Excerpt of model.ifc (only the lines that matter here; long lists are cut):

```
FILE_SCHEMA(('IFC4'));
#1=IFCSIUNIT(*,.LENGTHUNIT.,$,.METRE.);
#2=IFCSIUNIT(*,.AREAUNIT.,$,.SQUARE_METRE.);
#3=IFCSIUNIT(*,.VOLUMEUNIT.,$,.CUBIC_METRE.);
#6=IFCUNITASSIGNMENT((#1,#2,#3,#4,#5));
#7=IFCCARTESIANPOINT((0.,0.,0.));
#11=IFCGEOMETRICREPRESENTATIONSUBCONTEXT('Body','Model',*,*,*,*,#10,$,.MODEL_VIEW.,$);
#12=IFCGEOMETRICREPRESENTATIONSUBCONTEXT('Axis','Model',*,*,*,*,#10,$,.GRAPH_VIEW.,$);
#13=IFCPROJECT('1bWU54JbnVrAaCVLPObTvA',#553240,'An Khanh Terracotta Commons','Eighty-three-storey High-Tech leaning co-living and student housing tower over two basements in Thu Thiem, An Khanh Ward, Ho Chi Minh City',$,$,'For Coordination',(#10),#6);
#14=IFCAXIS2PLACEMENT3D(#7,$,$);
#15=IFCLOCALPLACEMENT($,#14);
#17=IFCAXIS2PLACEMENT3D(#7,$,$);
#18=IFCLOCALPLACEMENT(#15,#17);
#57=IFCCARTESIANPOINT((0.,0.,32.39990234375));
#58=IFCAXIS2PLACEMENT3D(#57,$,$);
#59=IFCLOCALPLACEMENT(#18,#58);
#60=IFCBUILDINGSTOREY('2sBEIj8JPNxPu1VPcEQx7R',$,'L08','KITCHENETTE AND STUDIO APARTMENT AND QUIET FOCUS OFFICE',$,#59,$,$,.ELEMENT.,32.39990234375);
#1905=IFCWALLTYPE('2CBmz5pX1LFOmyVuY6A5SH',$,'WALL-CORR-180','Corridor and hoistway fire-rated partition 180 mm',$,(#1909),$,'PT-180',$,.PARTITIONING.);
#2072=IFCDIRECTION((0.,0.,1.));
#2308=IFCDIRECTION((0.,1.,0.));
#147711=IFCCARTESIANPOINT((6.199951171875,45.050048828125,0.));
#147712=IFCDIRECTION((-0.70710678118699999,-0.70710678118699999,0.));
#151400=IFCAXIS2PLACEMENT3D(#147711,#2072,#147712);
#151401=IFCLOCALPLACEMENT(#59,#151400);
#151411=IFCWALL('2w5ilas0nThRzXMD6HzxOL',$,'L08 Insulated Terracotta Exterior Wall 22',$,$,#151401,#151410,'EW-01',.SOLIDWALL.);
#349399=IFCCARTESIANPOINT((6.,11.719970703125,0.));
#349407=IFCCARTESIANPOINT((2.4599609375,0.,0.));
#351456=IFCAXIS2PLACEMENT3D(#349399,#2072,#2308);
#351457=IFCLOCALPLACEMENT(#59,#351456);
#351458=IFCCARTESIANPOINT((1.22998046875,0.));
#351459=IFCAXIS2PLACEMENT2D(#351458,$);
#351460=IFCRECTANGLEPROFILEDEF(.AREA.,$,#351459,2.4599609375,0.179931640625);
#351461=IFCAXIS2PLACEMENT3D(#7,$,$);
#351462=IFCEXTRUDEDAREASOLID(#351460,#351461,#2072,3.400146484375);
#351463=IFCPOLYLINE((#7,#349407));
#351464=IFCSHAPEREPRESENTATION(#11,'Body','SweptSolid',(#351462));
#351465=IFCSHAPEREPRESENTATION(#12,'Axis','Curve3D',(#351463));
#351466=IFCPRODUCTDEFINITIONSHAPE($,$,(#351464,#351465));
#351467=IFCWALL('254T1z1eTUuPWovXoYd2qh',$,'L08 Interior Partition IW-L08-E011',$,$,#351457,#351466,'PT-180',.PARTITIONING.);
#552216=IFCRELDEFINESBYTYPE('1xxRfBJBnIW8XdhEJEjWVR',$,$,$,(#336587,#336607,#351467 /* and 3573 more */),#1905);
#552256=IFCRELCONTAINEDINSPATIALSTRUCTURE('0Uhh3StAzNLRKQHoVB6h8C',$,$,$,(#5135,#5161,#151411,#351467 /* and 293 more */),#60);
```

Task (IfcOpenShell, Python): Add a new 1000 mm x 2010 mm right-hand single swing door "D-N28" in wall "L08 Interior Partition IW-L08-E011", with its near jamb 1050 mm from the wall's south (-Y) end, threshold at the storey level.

```python
import numpy as np
import ifcopenshell
import ifcopenshell.api.feature
import ifcopenshell.api.geometry
import ifcopenshell.api.root
import ifcopenshell.api.spatial
import ifcopenshell.geom
import ifcopenshell.util.element
import ifcopenshell.util.placement
import ifcopenshell.util.representation
import ifcopenshell.util.shape
import ifcopenshell.util.unit

model = ifcopenshell.open("model.ifc")
unit_scale = ifcopenshell.util.unit.calculate_unit_scale(model)
settings = ifcopenshell.geom.settings()


def volume(element):
    """Net volume in cubic metres, openings subtracted."""
    shape = ifcopenshell.geom.create_shape(settings, element)
    return ifcopenshell.util.shape.get_volume(shape.geometry)


wall = model.by_guid("254T1z1eTUuPWovXoYd2qh")
storey = ifcopenshell.util.element.get_container(wall, ifc_class="IfcBuildingStorey")
context = ifcopenshell.util.representation.get_context(model, "Model", "Body", "MODEL_VIEW")
before = volume(wall)

width, height, from_end, sill = 1, 2.01, 1.05, 0.0  # metres

# The wall runs along its own X axis, and the end named is its -X end.
wall_shape = ifcopenshell.geom.create_shape(settings, wall)
x, y, z = ifcopenshell.util.shape.get_vertices(wall_shape.geometry).T
start = x.min() + from_end
face, thickness = float(y.min()), float(y.max() - y.min())
wall_matrix = ifcopenshell.util.placement.get_local_placement(wall.ObjectPlacement)
level = ifcopenshell.util.placement.get_local_placement(storey.ObjectPlacement)[2, 3]


def in_wall(x, y):
    """Placement at x, y metres in the wall's axes, at sill height."""
    matrix = wall_matrix.copy()
    matrix[:, 3] = wall_matrix @ np.array([x / unit_scale, y / unit_scale, 0.0, 1.0])
    matrix[2, 3] = level + sill / unit_scale
    return matrix


# Opening: a box that overshoots both wall faces by 50 mm.
opening = ifcopenshell.api.root.create_entity(model, ifc_class="IfcOpeningElement", predefined_type="OPENING")
box = ifcopenshell.api.geometry.add_wall_representation(
    model, context=context, length=width, height=height, thickness=thickness + 0.1
)
ifcopenshell.api.geometry.assign_representation(model, product=opening, representation=box)
ifcopenshell.api.geometry.edit_object_placement(model, product=opening, matrix=in_wall(start, face - 0.05), is_si=False)
ifcopenshell.api.feature.add_feature(model, feature=opening, element=wall)

door = ifcopenshell.api.root.create_entity(model, ifc_class="IfcDoor", name="D-N28", predefined_type="DOOR")
door.OverallWidth, door.OverallHeight = width / unit_scale, height / unit_scale
door.OperationType = "SINGLE_SWING_RIGHT"
body = ifcopenshell.api.geometry.add_door_representation(
    model,
    context=context,
    overall_width=door.OverallWidth,
    overall_height=door.OverallHeight,
    operation_type="SINGLE_SWING_RIGHT",
    lining_properties={"LiningDepth": thickness / unit_scale, "ThresholdDepth": thickness / unit_scale},
)
ifcopenshell.api.geometry.assign_representation(model, product=door, representation=body)
ifcopenshell.api.spatial.assign_container(model, products=[door], relating_structure=storey)
ifcopenshell.api.feature.add_filling(model, opening=opening, element=door)

# The lining spans the wall, so the door starts at the wall face.
ifcopenshell.api.geometry.edit_object_placement(model, product=door, matrix=in_wall(start, face), is_si=False)

after = volume(wall)

print(f"wall volume {before:.3f} -> {after:.3f} m3")

model.write("model-out.ifc")
```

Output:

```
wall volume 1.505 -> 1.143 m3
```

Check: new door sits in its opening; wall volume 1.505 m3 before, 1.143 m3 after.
